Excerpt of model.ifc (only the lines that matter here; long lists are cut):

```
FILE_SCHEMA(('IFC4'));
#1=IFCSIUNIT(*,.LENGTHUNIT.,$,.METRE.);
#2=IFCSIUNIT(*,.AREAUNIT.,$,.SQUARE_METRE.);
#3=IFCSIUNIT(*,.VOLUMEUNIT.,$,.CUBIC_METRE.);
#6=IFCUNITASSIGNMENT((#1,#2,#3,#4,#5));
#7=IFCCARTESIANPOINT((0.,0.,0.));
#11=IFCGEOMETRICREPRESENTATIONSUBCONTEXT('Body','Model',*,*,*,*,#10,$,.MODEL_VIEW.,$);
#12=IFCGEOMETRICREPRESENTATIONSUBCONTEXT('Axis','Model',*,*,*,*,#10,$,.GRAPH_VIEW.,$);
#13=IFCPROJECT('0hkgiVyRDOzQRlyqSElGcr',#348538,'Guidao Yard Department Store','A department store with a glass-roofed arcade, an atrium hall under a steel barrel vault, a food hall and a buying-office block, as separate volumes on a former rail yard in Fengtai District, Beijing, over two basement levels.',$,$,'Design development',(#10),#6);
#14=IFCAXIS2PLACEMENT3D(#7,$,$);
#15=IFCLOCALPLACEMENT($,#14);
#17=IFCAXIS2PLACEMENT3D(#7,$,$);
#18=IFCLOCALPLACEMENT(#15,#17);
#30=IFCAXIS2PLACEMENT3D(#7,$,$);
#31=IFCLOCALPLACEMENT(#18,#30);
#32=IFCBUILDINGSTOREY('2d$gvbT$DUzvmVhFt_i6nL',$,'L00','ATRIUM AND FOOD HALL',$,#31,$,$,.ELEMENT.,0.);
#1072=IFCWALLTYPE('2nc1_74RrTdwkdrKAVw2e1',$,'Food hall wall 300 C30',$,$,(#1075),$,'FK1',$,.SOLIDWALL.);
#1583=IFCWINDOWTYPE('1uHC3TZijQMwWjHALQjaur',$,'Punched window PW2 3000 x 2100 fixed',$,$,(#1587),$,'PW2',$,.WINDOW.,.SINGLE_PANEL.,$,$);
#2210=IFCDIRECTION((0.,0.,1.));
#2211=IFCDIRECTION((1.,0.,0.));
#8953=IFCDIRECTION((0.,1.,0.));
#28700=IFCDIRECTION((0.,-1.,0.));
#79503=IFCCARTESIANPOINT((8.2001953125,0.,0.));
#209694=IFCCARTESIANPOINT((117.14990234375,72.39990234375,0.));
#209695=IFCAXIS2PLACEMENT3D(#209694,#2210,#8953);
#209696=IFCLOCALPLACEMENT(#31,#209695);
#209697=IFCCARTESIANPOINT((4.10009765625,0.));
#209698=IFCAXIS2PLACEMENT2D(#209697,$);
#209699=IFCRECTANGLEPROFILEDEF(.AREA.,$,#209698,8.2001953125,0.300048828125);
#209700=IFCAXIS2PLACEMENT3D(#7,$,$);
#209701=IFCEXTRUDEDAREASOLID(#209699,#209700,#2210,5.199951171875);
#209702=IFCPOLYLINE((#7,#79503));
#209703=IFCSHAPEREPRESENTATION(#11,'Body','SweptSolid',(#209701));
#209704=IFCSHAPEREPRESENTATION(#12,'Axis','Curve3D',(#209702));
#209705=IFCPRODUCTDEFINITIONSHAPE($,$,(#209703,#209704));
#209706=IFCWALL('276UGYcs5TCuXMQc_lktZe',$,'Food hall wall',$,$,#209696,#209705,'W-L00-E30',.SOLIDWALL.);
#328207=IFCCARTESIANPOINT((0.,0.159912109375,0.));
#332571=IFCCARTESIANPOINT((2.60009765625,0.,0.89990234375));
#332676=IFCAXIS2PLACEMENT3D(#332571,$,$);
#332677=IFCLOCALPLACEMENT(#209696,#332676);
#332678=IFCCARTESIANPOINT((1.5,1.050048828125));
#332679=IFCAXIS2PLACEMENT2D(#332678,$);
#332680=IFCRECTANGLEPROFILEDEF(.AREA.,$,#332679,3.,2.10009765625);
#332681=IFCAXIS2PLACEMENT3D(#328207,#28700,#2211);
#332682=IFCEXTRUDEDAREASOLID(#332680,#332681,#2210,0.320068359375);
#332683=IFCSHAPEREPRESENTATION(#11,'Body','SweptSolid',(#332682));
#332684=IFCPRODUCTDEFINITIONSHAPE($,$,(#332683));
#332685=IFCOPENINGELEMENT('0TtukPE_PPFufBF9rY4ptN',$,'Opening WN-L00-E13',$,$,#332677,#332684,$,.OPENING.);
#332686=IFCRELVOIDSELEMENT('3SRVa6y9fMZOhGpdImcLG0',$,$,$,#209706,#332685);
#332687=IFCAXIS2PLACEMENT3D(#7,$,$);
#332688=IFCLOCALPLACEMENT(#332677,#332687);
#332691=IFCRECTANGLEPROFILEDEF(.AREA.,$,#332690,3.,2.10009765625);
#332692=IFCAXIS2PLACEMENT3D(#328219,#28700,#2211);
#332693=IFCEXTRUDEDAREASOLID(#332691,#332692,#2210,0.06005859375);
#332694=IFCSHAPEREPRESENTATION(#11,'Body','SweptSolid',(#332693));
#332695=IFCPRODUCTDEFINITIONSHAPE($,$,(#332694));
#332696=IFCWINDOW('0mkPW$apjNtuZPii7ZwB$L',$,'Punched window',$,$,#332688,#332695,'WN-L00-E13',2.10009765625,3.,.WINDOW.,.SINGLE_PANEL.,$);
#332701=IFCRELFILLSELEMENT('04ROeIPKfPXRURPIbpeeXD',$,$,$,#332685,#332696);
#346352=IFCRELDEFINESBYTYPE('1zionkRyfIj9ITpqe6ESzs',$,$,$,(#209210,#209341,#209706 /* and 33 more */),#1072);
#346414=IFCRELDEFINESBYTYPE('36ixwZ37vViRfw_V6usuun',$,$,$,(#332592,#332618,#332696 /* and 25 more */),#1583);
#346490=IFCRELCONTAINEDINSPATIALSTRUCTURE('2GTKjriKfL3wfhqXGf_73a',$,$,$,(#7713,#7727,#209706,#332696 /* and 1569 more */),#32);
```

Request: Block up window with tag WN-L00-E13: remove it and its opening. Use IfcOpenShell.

```python
import ifcopenshell
import ifcopenshell.api.feature
import ifcopenshell.api.root
import ifcopenshell.geom
import ifcopenshell.util.shape

model = ifcopenshell.open("model.ifc")
settings = ifcopenshell.geom.settings()


def volume(element):
    """Net volume in cubic metres, openings subtracted."""
    shape = ifcopenshell.geom.create_shape(settings, element)
    return ifcopenshell.util.shape.get_volume(shape.geometry)


window = model.by_guid("0mkPW$apjNtuZPii7ZwB$L")
opening = window.FillsVoids[0].RelatingOpeningElement
wall = opening.VoidsElements[0].RelatingBuildingElement
before = volume(wall)

ifcopenshell.api.root.remove_product(model, product=window)
ifcopenshell.api.feature.remove_feature(model, feature=opening)

after = volume(wall)

print(f"wall volume {before:.3f} -> {after:.3f} m3")

model.write("model_updated.ifc")
```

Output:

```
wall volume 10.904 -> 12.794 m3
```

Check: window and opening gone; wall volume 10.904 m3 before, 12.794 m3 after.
